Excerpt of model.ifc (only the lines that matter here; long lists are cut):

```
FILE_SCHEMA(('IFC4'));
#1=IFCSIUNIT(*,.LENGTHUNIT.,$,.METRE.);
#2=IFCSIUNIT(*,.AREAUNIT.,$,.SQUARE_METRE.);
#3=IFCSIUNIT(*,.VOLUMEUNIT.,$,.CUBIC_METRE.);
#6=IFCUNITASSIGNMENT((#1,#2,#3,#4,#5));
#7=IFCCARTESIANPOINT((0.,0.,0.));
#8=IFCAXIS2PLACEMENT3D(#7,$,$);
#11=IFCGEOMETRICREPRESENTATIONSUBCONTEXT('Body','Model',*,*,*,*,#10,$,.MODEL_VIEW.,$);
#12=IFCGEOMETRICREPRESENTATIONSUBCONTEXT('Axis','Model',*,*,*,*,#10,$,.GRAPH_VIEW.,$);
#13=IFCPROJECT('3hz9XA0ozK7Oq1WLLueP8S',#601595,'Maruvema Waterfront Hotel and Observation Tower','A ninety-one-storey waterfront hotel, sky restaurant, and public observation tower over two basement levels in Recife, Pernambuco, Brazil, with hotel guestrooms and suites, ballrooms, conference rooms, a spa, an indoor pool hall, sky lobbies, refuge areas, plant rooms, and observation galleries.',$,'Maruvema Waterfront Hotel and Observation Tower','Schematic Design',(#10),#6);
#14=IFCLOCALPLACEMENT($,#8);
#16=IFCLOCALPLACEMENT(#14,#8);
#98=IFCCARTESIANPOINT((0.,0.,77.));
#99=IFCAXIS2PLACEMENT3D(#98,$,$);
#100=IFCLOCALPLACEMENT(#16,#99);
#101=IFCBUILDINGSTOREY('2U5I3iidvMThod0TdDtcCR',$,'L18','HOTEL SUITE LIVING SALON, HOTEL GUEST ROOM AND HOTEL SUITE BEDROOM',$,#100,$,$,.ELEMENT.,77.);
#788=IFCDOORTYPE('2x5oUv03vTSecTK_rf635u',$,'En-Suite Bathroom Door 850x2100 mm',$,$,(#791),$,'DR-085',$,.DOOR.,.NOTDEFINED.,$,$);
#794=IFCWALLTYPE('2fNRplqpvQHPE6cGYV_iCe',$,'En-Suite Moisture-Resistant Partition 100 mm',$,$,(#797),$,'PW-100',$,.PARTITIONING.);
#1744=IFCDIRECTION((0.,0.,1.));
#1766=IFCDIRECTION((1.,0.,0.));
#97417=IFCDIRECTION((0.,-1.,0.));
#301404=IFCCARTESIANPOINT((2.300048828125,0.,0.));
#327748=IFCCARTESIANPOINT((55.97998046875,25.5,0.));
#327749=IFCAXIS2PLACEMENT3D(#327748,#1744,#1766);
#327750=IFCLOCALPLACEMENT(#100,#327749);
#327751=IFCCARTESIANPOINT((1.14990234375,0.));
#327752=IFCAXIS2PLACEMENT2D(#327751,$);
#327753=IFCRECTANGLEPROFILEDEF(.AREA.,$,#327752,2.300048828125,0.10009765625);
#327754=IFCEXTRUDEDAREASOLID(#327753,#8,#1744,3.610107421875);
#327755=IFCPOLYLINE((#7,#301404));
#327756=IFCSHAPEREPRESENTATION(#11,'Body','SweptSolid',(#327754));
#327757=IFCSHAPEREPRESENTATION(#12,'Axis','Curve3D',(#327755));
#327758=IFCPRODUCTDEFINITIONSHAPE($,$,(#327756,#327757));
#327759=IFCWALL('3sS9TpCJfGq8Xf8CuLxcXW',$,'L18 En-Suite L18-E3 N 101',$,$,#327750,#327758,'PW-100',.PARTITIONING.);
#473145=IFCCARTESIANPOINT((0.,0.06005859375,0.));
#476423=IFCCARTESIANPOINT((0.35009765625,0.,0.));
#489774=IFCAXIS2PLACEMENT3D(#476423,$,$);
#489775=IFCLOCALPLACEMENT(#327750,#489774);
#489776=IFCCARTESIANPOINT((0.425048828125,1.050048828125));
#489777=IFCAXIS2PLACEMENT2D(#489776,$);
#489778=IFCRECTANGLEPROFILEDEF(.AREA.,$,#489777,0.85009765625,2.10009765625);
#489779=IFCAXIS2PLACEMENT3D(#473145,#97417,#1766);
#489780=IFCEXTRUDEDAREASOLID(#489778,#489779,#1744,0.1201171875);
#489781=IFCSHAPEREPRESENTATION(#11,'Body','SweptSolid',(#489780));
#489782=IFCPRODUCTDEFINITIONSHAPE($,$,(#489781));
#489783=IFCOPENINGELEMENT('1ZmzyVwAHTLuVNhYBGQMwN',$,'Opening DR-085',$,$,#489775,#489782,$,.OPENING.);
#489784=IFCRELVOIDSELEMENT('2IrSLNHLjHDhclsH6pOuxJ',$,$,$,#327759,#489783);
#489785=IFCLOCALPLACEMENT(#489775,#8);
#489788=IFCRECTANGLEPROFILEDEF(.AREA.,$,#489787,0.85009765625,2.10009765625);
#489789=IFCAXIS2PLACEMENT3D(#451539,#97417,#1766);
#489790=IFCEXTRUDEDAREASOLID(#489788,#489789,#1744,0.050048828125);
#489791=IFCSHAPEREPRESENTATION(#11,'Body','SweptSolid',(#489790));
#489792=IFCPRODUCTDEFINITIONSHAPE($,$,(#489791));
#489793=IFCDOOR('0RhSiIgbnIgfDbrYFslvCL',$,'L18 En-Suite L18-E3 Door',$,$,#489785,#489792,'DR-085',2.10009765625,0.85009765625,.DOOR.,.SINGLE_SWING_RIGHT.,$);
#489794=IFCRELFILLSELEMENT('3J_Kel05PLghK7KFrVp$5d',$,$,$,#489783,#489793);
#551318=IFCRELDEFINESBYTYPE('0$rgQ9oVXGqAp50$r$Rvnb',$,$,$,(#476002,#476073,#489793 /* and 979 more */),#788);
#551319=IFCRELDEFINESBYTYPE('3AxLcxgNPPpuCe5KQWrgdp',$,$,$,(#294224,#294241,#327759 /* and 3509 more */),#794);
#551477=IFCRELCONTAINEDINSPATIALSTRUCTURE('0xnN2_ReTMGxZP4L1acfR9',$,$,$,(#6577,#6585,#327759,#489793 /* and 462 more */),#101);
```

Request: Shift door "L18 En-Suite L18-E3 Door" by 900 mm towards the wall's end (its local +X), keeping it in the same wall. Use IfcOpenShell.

```python
import ifcopenshell
import ifcopenshell.api.geometry
import ifcopenshell.util.placement

model = ifcopenshell.open("model.ifc")

door = model.by_guid("0RhSiIgbnIgfDbrYFslvCL")
opening = door.FillsVoids[0].RelatingOpeningElement
wall = opening.VoidsElements[0].RelatingBuildingElement

wall_matrix = ifcopenshell.util.placement.get_local_placement(wall.ObjectPlacement)
shift = wall_matrix[:3, 0] * 0.9
before = ifcopenshell.util.placement.get_local_placement(door.ObjectPlacement)[:3, 3].copy()

# The door is placed relative to its opening, so it follows when the opening moves.
matrix = ifcopenshell.util.placement.get_local_placement(opening.ObjectPlacement)
matrix[:3, 3] += shift
ifcopenshell.api.geometry.edit_object_placement(
    model, product=opening, matrix=matrix, is_si=False, should_transform_children=True
)

after = ifcopenshell.util.placement.get_local_placement(door.ObjectPlacement)[:3, 3]
print("door moved by", (after - before).round(3) + 0.0)

model.write("model_updated.ifc")
```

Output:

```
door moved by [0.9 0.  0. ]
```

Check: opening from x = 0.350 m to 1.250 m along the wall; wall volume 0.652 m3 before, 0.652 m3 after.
